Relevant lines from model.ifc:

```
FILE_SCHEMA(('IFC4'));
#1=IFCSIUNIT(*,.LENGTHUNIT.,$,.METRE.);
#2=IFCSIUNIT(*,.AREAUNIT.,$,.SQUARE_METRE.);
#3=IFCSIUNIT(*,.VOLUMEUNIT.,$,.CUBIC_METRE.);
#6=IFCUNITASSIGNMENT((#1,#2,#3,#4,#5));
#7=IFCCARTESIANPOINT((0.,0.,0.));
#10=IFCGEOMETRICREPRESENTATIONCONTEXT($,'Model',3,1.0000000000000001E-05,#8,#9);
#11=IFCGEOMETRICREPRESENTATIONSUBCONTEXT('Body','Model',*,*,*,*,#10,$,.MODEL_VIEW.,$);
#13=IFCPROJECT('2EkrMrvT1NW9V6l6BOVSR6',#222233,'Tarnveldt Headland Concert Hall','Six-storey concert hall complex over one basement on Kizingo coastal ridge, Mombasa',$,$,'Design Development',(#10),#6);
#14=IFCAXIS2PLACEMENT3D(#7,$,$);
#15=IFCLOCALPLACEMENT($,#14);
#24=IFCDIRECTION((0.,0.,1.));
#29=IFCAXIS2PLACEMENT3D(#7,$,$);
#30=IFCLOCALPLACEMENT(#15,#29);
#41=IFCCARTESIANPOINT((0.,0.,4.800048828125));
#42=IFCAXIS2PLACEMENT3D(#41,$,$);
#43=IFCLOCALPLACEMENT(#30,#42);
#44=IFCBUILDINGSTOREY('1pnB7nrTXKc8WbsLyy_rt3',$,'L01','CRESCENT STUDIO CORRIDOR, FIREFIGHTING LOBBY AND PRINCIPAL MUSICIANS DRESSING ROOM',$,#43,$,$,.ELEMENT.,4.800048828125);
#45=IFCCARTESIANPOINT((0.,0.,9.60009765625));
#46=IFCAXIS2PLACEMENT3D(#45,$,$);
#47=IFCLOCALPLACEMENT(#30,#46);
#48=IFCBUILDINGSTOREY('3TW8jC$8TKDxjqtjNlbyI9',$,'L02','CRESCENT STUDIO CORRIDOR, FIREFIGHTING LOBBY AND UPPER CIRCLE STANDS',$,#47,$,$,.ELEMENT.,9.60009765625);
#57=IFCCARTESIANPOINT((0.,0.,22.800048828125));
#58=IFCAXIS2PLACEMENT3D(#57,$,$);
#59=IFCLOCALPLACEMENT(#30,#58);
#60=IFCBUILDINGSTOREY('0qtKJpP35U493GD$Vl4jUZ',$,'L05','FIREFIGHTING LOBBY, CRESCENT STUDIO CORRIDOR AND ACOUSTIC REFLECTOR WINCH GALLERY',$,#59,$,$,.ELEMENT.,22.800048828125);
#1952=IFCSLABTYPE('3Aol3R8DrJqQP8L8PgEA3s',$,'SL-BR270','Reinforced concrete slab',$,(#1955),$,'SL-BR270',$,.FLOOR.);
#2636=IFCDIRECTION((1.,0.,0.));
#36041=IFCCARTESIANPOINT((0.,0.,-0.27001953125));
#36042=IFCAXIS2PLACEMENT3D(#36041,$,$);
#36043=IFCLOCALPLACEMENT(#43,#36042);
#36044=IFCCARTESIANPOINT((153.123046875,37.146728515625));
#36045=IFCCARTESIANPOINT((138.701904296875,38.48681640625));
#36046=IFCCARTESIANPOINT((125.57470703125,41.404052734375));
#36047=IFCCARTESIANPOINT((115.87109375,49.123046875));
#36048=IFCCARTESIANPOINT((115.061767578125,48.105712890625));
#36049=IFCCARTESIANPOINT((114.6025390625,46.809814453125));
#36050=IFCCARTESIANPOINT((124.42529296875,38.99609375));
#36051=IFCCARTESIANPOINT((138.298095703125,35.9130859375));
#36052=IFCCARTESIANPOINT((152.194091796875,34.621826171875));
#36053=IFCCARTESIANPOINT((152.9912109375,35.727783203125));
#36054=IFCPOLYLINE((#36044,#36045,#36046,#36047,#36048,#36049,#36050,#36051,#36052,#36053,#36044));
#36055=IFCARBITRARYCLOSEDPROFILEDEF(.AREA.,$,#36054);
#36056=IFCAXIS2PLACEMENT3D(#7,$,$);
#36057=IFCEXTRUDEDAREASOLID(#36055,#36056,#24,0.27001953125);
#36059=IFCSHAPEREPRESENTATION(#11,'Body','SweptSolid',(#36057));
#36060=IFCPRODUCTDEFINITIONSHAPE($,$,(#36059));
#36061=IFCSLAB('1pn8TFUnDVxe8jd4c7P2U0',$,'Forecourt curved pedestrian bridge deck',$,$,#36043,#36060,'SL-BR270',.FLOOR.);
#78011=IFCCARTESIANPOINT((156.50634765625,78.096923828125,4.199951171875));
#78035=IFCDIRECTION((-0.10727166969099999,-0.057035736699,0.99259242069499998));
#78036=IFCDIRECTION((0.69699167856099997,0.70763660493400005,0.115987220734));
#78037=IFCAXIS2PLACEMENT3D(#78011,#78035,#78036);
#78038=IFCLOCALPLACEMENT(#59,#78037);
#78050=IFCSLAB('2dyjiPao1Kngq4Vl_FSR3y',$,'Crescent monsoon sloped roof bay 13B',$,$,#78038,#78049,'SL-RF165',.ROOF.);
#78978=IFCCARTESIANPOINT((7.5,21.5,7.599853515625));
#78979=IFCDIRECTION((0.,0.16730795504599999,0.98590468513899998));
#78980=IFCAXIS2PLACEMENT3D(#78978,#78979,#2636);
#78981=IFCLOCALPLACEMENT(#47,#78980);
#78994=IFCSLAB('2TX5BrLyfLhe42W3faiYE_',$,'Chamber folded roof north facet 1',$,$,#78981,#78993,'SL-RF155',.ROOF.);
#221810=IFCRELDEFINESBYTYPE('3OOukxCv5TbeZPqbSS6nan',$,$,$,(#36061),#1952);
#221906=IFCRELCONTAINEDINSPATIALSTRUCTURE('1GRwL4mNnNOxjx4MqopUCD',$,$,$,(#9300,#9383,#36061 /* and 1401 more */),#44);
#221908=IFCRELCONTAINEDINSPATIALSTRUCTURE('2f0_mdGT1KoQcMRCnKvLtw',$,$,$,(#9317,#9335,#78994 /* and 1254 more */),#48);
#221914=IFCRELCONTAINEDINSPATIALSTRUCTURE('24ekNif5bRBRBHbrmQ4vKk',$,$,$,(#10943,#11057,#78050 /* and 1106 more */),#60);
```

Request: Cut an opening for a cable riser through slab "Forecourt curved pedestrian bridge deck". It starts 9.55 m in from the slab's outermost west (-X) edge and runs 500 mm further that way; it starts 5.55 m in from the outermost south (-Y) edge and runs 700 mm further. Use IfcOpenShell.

```python
import numpy as np
import ifcopenshell
import ifcopenshell.api.feature
import ifcopenshell.api.geometry
import ifcopenshell.api.root
import ifcopenshell.geom
import ifcopenshell.util.placement
import ifcopenshell.util.representation
import ifcopenshell.util.shape
import ifcopenshell.util.unit

model = ifcopenshell.open("model.ifc")
unit_scale = ifcopenshell.util.unit.calculate_unit_scale(model)
settings = ifcopenshell.geom.settings()


def volume(element):
    """Net volume in cubic metres, openings subtracted."""
    shape = ifcopenshell.geom.create_shape(settings, element)
    return ifcopenshell.util.shape.get_volume(shape.geometry)


slab = model.by_guid("1pn8TFUnDVxe8jd4c7P2U0")
before = volume(slab)

# Extent in the slab's own axes, in metres. The edges named are its -X and -Y sides.
slab_shape = ifcopenshell.geom.create_shape(settings, slab)
vertices = ifcopenshell.util.shape.get_vertices(slab_shape.geometry)
x_min, y_min, bottom = vertices.min(axis=0)
top = vertices[:, 2].max()

opening = ifcopenshell.api.root.create_entity(model, ifc_class="IfcOpeningElement", name="Cable riser opening", predefined_type="OPENING")
context = ifcopenshell.util.representation.get_context(model, "Model", "Body", "MODEL_VIEW")
width, depth = 0.5, 0.7
outline = [(0.0, 0.0), (width, 0.0), (width, depth), (0.0, depth), (0.0, 0.0)]
# Overshoot both faces by 50 mm so the cut is clean.
shape = ifcopenshell.api.geometry.add_slab_representation(
    model, context=context, depth=top - bottom + 0.1, polyline=outline
)
ifcopenshell.api.geometry.assign_representation(model, product=opening, representation=shape)

matrix = ifcopenshell.util.placement.get_local_placement(slab.ObjectPlacement)
matrix[:, 3] = matrix @ np.append(np.array([x_min + 9.55, y_min + 5.55, bottom - 0.05]) / unit_scale, 1.0)
ifcopenshell.api.geometry.edit_object_placement(model, product=opening, matrix=matrix, is_si=False)
ifcopenshell.api.feature.add_feature(model, feature=opening, element=slab)

after = volume(slab)

print(f"slab volume {before:.3f} -> {after:.3f} m3")

model.write("model_edited.ifc")
```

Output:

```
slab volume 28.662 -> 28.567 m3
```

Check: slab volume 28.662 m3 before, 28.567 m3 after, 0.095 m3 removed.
